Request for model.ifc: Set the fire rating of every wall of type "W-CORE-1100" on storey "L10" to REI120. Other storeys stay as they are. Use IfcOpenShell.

First a look at what the model holds.

```python
import ifcopenshell
import ifcopenshell.util.element

model = ifcopenshell.open("model.ifc")
print(model.schema)
storey = next(s for s in model.by_type("IfcBuildingStorey") if s.Name == "L10")
walls = [e for e in ifcopenshell.util.element.get_decomposition(storey) if e.is_a("IfcWall")]
seen = {}
for e in walls:
    element_type = ifcopenshell.util.element.get_type(e)
    key = (element_type.Name if element_type != e and element_type else None, ifcopenshell.util.element.get_pset(e, "Pset_WallCommon", "FireRating"))
    seen[key] = seen.get(key, 0) + 1
for (name, value), count in sorted(seen.items(), key=str):
    print(count, "x", name, "|", value)
```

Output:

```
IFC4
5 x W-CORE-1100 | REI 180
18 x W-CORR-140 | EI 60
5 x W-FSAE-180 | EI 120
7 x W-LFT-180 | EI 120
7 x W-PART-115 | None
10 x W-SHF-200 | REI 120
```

```python
import ifcopenshell
import ifcopenshell.api.pset
import ifcopenshell.util.element

model = ifcopenshell.open("model.ifc")

storey = next(s for s in model.by_type("IfcBuildingStorey") if s.Name == "L10")
walls = [e for e in ifcopenshell.util.element.get_decomposition(storey) if e.is_a("IfcWall")]

count = 0
for e in walls:
    element_type = ifcopenshell.util.element.get_type(e)
    if element_type in (None, e) or element_type.Name != "W-CORE-1100":
        continue
    found = ifcopenshell.util.element.get_pset(e, "Pset_WallCommon", should_inherit=False)
    if found:
        pset = model.by_id(found["id"])
        if len(ifcopenshell.util.element.get_elements_by_pset(pset)) > 1:
            pset = ifcopenshell.api.pset.unshare_pset(model, products=[e], pset=pset)[0]
    else:
        pset = ifcopenshell.api.pset.add_pset(model, product=e, name="Pset_WallCommon")
    ifcopenshell.api.pset.edit_pset(model, pset=pset, properties={"FireRating": "REI120"})
    count += 1

print(count, "walls updated")

model.write("model-out.ifc")
```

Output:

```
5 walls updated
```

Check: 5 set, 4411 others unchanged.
